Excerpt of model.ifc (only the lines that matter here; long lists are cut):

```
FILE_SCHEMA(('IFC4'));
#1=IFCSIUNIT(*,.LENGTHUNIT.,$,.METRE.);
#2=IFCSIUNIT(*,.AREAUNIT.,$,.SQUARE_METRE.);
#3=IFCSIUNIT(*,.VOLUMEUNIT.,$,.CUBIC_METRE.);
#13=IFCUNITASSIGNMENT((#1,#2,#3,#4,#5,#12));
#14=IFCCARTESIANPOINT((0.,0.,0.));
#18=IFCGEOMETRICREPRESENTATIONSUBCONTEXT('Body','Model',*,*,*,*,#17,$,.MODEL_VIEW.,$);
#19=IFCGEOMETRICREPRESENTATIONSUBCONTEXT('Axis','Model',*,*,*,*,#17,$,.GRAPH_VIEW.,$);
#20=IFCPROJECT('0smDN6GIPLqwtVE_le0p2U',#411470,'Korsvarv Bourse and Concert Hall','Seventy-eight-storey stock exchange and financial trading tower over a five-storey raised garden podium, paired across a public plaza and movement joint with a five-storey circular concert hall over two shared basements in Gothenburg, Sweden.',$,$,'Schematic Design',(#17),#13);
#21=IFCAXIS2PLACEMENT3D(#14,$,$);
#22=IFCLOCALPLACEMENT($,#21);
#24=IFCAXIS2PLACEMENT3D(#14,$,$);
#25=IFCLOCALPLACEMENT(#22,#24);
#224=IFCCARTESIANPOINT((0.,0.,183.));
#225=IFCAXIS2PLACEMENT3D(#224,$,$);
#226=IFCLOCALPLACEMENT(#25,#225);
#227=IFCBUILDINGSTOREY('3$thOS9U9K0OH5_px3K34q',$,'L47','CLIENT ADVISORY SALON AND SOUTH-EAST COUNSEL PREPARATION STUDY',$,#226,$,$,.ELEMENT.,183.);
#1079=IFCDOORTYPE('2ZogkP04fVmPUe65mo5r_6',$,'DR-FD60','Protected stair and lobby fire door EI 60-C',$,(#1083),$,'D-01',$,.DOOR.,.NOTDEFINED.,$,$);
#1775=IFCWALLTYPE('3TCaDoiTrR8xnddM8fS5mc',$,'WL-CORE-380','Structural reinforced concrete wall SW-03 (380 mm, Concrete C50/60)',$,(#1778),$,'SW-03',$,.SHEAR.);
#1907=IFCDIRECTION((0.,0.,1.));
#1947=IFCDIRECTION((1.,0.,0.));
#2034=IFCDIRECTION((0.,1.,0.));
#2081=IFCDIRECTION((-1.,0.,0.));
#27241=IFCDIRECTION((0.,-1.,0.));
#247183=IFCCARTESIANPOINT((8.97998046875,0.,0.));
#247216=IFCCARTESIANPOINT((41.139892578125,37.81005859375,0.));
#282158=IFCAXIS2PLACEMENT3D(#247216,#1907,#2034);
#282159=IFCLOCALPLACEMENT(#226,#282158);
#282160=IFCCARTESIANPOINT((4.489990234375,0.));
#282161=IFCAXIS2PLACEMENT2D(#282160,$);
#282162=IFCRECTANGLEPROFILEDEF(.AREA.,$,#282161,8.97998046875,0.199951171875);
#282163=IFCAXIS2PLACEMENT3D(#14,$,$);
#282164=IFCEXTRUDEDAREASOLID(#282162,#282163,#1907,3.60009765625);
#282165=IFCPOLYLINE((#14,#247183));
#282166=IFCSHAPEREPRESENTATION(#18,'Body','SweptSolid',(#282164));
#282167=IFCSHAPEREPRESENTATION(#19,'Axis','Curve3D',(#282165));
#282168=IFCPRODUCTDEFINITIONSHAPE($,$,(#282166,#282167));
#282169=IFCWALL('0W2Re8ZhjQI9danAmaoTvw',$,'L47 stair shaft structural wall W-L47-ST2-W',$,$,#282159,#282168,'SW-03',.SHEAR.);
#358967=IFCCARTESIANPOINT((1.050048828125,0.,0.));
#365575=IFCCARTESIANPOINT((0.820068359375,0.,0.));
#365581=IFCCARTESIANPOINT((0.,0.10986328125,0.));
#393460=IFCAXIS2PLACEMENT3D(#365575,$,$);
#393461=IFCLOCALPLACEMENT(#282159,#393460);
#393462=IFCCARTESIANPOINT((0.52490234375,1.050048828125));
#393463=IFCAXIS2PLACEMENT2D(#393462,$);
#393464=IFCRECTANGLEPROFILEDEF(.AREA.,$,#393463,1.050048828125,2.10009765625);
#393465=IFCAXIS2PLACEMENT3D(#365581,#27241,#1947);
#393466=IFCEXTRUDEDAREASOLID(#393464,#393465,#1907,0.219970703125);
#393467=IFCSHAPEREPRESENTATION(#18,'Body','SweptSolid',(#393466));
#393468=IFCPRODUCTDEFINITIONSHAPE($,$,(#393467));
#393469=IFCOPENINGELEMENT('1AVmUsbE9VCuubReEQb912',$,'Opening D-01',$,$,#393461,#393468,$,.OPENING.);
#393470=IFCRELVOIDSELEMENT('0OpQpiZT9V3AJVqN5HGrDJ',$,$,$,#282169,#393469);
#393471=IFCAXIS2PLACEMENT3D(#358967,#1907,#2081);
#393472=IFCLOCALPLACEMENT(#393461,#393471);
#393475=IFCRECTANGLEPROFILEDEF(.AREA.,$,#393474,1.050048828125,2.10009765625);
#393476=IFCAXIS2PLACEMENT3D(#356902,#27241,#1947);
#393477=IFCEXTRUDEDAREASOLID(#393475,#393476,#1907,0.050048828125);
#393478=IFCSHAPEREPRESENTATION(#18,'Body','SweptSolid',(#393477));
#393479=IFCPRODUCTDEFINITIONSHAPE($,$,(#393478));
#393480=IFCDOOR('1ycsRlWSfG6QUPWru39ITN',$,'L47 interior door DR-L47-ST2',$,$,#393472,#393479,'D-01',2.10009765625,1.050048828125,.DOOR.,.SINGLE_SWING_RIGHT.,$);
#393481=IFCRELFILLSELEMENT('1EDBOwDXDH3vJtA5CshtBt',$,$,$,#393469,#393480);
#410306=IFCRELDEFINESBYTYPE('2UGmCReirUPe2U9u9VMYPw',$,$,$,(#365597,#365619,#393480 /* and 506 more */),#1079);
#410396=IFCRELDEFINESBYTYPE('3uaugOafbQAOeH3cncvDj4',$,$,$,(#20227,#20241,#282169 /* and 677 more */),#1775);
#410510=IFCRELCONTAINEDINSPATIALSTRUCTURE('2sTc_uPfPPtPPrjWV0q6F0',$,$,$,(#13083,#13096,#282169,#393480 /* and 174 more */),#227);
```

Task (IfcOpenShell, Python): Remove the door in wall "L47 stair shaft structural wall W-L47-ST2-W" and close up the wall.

```python
import ifcopenshell
import ifcopenshell.api.feature
import ifcopenshell.api.root
import ifcopenshell.geom
import ifcopenshell.util.shape

model = ifcopenshell.open("model.ifc")
settings = ifcopenshell.geom.settings()


def volume(element):
    """Net volume in cubic metres, openings subtracted."""
    shape = ifcopenshell.geom.create_shape(settings, element)
    return ifcopenshell.util.shape.get_volume(shape.geometry)


door = model.by_guid("1ycsRlWSfG6QUPWru39ITN")
opening = door.FillsVoids[0].RelatingOpeningElement
wall = opening.VoidsElements[0].RelatingBuildingElement
before = volume(wall)

ifcopenshell.api.root.remove_product(model, product=door)
ifcopenshell.api.feature.remove_feature(model, feature=opening)

after = volume(wall)

print(f"wall volume {before:.3f} -> {after:.3f} m3")

model.write("model_v2.ifc")
```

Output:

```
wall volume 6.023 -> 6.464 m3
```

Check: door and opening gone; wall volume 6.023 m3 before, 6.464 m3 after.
